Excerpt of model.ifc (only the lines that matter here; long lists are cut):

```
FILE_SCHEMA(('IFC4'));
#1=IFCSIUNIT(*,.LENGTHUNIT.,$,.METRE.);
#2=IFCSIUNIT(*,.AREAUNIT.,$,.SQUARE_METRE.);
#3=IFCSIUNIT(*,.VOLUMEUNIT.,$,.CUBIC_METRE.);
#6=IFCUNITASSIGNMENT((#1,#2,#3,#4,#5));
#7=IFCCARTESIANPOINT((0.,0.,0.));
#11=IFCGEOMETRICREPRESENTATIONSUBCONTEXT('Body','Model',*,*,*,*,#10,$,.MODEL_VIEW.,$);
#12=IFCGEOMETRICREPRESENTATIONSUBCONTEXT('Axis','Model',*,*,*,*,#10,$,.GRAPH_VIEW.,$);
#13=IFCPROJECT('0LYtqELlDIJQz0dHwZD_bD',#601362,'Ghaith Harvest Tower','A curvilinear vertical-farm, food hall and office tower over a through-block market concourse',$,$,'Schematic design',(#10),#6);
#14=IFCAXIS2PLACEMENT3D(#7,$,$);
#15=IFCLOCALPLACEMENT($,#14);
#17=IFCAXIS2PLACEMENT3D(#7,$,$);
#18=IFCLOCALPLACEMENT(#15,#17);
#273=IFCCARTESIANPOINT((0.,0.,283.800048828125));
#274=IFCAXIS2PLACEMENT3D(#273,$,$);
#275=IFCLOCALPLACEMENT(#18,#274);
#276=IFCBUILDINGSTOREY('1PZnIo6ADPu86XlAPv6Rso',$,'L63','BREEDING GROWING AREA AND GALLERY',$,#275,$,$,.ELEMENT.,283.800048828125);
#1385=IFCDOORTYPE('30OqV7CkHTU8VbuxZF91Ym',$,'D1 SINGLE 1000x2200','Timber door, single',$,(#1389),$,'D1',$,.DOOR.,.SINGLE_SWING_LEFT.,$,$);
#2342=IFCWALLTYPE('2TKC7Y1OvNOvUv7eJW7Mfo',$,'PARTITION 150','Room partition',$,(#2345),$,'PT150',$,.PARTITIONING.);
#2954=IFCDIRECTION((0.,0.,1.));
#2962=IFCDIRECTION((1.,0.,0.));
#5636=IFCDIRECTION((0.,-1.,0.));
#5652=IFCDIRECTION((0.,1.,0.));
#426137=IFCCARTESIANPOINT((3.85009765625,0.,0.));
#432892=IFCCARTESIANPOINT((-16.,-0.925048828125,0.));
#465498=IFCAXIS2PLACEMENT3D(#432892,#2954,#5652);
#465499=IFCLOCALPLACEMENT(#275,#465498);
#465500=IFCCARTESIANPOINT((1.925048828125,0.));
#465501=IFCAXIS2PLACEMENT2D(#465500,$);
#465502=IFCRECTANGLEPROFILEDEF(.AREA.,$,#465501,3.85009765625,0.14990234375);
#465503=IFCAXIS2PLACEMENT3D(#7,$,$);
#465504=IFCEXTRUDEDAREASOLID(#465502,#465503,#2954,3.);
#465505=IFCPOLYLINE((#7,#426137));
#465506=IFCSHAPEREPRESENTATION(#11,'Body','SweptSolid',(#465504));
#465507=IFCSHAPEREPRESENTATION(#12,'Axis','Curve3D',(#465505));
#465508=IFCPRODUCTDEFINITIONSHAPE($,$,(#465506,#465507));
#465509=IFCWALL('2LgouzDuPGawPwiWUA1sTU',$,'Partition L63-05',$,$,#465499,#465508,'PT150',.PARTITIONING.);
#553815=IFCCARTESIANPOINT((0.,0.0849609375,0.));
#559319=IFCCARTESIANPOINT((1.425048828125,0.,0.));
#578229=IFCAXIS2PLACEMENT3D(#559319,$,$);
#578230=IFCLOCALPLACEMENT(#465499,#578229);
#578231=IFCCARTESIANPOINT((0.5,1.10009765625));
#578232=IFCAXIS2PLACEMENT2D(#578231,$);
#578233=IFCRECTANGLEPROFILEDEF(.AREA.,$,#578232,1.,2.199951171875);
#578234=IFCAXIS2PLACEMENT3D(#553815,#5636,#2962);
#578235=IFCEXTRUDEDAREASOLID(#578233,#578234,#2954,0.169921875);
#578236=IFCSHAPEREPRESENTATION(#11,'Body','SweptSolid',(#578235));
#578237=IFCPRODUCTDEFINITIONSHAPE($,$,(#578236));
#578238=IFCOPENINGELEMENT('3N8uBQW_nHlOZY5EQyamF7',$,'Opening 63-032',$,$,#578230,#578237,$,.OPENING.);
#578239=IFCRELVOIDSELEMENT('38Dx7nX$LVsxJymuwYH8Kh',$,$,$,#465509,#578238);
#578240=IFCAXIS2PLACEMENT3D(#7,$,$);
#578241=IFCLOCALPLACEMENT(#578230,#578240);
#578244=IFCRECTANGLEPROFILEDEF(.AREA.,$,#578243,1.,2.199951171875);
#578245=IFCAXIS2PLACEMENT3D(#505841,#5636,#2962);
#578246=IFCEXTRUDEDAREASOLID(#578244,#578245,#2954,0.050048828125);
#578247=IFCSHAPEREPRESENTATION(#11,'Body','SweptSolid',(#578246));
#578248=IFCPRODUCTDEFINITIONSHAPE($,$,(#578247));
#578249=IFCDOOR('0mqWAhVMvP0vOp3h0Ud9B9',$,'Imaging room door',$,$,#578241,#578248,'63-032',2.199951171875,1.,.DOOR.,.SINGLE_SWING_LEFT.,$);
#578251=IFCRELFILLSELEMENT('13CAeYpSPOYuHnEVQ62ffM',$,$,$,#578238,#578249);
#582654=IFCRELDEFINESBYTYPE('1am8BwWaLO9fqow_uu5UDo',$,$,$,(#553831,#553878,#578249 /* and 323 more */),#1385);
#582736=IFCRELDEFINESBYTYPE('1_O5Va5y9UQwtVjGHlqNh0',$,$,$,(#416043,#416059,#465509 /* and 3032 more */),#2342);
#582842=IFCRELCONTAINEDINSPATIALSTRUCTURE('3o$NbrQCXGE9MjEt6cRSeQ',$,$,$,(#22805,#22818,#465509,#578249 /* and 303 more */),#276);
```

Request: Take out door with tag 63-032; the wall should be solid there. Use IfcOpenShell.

```python
import ifcopenshell
import ifcopenshell.api.feature
import ifcopenshell.api.root
import ifcopenshell.geom
import ifcopenshell.util.shape

model = ifcopenshell.open("model.ifc")
settings = ifcopenshell.geom.settings()


def volume(element):
    """Net volume in cubic metres, openings subtracted."""
    shape = ifcopenshell.geom.create_shape(settings, element)
    return ifcopenshell.util.shape.get_volume(shape.geometry)


door = model.by_guid("0mqWAhVMvP0vOp3h0Ud9B9")
opening = door.FillsVoids[0].RelatingOpeningElement
wall = opening.VoidsElements[0].RelatingBuildingElement
before = volume(wall)

ifcopenshell.api.root.remove_product(model, product=door)
ifcopenshell.api.feature.remove_feature(model, feature=opening)

after = volume(wall)

print(f"wall volume {before:.3f} -> {after:.3f} m3")

model.write("model_updated.ifc")
```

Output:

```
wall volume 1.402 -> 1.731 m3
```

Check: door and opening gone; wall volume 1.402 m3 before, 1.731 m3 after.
